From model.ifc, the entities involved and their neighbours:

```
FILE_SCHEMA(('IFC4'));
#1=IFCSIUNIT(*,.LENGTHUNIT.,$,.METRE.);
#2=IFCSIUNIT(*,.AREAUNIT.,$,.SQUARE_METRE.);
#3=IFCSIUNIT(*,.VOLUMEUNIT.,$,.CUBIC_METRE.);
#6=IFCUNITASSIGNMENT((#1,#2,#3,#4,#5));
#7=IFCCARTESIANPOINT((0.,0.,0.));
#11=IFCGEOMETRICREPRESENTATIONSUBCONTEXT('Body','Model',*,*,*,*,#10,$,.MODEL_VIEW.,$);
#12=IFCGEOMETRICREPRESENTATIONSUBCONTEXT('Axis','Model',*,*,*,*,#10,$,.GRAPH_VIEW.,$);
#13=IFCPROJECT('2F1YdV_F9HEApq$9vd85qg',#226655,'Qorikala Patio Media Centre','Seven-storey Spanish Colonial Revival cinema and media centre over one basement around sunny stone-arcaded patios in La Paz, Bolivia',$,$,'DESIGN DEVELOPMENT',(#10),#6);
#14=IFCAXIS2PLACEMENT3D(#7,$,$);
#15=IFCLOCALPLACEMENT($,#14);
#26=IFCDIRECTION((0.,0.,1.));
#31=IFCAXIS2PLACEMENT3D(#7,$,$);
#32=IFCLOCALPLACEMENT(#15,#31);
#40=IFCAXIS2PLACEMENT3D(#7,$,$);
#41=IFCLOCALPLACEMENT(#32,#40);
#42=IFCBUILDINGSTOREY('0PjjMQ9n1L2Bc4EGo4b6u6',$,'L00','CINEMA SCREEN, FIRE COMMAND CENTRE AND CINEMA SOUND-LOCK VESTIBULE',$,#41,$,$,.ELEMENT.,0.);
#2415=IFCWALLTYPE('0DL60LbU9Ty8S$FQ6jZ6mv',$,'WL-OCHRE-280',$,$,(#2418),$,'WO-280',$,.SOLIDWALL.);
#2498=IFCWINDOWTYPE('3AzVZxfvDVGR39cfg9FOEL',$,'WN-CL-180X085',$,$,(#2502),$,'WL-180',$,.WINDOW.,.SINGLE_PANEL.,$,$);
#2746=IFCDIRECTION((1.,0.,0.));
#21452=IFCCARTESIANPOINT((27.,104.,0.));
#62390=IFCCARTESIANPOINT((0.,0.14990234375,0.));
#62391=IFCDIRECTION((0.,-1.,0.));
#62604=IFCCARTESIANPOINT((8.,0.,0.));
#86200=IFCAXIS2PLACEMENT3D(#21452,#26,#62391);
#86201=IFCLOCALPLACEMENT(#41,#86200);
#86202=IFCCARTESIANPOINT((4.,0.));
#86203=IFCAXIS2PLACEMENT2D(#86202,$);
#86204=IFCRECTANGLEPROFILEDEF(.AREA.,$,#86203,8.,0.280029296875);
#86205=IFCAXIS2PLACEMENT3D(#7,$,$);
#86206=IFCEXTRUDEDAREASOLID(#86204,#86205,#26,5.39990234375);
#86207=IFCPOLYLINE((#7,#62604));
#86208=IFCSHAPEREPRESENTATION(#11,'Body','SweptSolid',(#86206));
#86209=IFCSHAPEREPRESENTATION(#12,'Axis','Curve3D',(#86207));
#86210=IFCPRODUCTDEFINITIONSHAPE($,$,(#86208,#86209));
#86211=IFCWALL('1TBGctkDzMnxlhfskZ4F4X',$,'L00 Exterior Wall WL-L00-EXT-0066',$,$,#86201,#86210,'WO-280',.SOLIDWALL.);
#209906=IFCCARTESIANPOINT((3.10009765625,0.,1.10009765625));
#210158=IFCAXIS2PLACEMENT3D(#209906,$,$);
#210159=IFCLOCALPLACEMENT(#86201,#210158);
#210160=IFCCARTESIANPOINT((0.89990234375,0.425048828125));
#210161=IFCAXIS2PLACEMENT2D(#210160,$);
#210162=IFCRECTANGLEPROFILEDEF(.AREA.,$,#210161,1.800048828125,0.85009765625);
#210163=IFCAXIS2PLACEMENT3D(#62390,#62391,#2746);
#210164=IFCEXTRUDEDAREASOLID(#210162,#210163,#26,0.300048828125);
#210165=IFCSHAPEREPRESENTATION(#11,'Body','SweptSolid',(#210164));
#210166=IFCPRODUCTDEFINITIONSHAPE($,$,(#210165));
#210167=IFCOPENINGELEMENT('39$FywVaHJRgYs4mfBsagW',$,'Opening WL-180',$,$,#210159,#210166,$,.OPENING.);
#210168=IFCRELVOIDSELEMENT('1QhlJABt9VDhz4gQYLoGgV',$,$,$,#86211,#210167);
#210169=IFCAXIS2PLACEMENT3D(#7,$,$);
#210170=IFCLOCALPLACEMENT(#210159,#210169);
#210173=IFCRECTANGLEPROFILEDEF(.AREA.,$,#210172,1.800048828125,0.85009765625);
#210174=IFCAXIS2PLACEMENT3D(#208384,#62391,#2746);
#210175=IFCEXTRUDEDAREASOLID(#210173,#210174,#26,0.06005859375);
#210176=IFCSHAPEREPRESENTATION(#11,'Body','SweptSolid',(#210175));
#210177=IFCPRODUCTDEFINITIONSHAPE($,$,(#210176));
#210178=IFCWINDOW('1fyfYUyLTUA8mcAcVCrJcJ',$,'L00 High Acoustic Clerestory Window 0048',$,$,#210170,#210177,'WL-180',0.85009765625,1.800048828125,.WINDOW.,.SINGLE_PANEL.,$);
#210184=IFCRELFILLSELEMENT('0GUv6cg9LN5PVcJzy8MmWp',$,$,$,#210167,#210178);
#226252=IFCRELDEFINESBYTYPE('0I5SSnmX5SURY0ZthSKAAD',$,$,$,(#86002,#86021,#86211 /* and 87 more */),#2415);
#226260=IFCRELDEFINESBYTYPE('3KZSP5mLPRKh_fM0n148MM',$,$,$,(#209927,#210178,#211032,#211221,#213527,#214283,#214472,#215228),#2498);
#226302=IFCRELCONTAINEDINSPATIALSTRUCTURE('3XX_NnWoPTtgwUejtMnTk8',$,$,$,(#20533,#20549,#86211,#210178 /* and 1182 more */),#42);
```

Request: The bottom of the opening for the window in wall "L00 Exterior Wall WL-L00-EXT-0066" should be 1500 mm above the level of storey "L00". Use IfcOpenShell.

```python
import numpy as np
import ifcopenshell
import ifcopenshell.api.geometry
import ifcopenshell.geom
import ifcopenshell.util.element
import ifcopenshell.util.placement
import ifcopenshell.util.shape
import ifcopenshell.util.unit

model = ifcopenshell.open("model.ifc")
unit_scale = ifcopenshell.util.unit.calculate_unit_scale(model)

window = model.by_id(210178)
opening = window.FillsVoids[0].RelatingOpeningElement
storey = ifcopenshell.util.element.get_container(window, ifc_class="IfcBuildingStorey")
level = ifcopenshell.util.placement.get_local_placement(storey.ObjectPlacement)[2, 3]

# The opening's origin need not be at the sill, so measure its lowest point.
shape = ifcopenshell.geom.create_shape(ifcopenshell.geom.settings(), opening)
bottom = ifcopenshell.util.shape.get_shape_bottom_elevation(shape, shape.geometry) / unit_scale
dz = level + 1.5 - bottom

shift = np.array([0.0, 0.0, dz])
# The window is placed relative to its opening, so it follows when the opening moves.
matrix = ifcopenshell.util.placement.get_local_placement(opening.ObjectPlacement)
matrix[:3, 3] += shift
ifcopenshell.api.geometry.edit_object_placement(
    model, product=opening, matrix=matrix, is_si=False, should_transform_children=True
)

print(f"moved by {dz * unit_scale:+.3f} m")

model.write("model_edited.ifc")
```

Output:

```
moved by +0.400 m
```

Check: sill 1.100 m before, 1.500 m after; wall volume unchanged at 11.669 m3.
